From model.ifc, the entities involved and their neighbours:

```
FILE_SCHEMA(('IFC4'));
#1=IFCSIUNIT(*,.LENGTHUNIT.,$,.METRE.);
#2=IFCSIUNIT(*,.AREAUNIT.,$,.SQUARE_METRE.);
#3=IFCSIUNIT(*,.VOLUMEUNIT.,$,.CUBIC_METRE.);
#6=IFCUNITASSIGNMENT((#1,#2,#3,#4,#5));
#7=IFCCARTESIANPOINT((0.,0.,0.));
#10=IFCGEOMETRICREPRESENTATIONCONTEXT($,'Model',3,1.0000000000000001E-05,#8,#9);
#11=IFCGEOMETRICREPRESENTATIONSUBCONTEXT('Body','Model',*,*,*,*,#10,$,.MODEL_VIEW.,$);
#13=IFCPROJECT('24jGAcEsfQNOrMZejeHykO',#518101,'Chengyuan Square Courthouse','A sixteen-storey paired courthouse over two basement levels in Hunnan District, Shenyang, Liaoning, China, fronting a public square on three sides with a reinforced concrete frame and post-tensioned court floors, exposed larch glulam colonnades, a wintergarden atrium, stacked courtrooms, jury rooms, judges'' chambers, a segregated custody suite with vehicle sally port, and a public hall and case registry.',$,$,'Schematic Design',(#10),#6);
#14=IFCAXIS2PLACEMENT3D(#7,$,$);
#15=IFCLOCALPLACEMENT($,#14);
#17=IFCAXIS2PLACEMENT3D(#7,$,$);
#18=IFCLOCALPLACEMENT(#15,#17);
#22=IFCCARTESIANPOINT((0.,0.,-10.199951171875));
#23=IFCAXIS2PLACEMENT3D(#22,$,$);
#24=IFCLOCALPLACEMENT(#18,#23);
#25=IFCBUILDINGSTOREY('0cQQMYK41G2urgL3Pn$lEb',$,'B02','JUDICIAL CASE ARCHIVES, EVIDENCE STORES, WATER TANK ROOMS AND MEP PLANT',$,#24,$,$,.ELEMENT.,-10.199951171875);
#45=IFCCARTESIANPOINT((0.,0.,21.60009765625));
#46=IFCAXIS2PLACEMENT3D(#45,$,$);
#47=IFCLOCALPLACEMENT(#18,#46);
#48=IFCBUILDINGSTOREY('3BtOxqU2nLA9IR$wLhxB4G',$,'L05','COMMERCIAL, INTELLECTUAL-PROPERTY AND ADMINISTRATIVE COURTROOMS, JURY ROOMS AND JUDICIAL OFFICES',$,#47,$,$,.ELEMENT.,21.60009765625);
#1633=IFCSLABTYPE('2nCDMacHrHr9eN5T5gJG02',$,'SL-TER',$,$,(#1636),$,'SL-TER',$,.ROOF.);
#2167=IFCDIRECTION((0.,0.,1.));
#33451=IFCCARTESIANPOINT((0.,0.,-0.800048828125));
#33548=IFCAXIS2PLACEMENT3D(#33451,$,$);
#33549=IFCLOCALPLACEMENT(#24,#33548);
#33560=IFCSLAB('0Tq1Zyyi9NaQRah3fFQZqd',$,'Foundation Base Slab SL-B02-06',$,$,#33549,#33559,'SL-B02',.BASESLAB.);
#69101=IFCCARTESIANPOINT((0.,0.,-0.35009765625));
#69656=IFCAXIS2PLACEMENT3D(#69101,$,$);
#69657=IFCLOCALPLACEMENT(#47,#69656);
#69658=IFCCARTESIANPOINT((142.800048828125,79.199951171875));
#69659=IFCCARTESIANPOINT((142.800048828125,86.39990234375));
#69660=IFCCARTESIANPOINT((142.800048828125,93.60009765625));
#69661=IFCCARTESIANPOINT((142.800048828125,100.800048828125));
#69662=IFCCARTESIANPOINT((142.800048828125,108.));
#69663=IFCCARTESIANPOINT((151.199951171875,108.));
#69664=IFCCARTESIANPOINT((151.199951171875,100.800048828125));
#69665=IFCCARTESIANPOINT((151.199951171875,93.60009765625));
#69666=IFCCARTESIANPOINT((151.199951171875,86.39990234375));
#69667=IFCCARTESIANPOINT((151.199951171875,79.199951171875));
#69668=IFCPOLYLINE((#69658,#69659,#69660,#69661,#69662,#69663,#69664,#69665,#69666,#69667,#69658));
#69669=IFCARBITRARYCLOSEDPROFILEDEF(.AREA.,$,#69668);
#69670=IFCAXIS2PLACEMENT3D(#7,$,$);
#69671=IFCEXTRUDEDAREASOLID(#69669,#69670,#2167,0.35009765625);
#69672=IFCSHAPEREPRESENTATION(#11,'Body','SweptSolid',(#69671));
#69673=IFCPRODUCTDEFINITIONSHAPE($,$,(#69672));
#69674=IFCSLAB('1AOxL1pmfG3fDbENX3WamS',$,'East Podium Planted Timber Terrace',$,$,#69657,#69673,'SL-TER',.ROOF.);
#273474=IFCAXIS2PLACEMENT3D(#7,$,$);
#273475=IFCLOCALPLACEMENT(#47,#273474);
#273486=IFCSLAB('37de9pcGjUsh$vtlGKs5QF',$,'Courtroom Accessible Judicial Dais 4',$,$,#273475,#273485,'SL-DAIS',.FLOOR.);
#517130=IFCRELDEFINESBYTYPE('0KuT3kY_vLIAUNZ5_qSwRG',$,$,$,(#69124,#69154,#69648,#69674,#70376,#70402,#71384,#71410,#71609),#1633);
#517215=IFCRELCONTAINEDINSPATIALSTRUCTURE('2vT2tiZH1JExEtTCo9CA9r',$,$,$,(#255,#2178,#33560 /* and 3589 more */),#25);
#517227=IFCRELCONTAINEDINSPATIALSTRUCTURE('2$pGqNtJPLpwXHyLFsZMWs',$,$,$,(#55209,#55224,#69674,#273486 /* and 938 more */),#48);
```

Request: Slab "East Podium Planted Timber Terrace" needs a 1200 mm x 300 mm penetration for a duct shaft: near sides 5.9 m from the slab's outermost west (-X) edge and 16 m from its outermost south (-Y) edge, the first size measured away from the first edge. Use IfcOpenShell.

```python
import numpy as np
import ifcopenshell
import ifcopenshell.api.feature
import ifcopenshell.api.geometry
import ifcopenshell.api.root
import ifcopenshell.geom
import ifcopenshell.util.placement
import ifcopenshell.util.representation
import ifcopenshell.util.shape
import ifcopenshell.util.unit

model = ifcopenshell.open("model.ifc")
unit_scale = ifcopenshell.util.unit.calculate_unit_scale(model)
settings = ifcopenshell.geom.settings()


def volume(element):
    """Net volume in cubic metres, openings subtracted."""
    shape = ifcopenshell.geom.create_shape(settings, element)
    return ifcopenshell.util.shape.get_volume(shape.geometry)


slab = model.by_id(69674)
before = volume(slab)

# Extent in the slab's own axes, in metres. The edges named are its -X and -Y sides.
slab_shape = ifcopenshell.geom.create_shape(settings, slab)
vertices = ifcopenshell.util.shape.get_vertices(slab_shape.geometry)
x_min, y_min, bottom = vertices.min(axis=0)
top = vertices[:, 2].max()

opening = ifcopenshell.api.root.create_entity(model, ifc_class="IfcOpeningElement", name="Duct shaft opening", predefined_type="OPENING")
context = ifcopenshell.util.representation.get_context(model, "Model", "Body", "MODEL_VIEW")
width, depth = 1.2, 0.3
outline = [(0.0, 0.0), (width, 0.0), (width, depth), (0.0, depth), (0.0, 0.0)]
# Overshoot both faces by 50 mm so the cut is clean.
shape = ifcopenshell.api.geometry.add_slab_representation(
    model, context=context, depth=top - bottom + 0.1, polyline=outline
)
ifcopenshell.api.geometry.assign_representation(model, product=opening, representation=shape)

matrix = ifcopenshell.util.placement.get_local_placement(slab.ObjectPlacement)
matrix[:, 3] = matrix @ np.append(np.array([x_min + 5.9, y_min + 16, bottom - 0.05]) / unit_scale, 1.0)
ifcopenshell.api.geometry.edit_object_placement(model, product=opening, matrix=matrix, is_si=False)
ifcopenshell.api.feature.add_feature(model, feature=opening, element=slab)

after = volume(slab)

print(f"slab volume {before:.3f} -> {after:.3f} m3")

model.write("model_v2.ifc")
```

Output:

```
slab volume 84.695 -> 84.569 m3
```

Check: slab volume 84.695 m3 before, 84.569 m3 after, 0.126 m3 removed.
